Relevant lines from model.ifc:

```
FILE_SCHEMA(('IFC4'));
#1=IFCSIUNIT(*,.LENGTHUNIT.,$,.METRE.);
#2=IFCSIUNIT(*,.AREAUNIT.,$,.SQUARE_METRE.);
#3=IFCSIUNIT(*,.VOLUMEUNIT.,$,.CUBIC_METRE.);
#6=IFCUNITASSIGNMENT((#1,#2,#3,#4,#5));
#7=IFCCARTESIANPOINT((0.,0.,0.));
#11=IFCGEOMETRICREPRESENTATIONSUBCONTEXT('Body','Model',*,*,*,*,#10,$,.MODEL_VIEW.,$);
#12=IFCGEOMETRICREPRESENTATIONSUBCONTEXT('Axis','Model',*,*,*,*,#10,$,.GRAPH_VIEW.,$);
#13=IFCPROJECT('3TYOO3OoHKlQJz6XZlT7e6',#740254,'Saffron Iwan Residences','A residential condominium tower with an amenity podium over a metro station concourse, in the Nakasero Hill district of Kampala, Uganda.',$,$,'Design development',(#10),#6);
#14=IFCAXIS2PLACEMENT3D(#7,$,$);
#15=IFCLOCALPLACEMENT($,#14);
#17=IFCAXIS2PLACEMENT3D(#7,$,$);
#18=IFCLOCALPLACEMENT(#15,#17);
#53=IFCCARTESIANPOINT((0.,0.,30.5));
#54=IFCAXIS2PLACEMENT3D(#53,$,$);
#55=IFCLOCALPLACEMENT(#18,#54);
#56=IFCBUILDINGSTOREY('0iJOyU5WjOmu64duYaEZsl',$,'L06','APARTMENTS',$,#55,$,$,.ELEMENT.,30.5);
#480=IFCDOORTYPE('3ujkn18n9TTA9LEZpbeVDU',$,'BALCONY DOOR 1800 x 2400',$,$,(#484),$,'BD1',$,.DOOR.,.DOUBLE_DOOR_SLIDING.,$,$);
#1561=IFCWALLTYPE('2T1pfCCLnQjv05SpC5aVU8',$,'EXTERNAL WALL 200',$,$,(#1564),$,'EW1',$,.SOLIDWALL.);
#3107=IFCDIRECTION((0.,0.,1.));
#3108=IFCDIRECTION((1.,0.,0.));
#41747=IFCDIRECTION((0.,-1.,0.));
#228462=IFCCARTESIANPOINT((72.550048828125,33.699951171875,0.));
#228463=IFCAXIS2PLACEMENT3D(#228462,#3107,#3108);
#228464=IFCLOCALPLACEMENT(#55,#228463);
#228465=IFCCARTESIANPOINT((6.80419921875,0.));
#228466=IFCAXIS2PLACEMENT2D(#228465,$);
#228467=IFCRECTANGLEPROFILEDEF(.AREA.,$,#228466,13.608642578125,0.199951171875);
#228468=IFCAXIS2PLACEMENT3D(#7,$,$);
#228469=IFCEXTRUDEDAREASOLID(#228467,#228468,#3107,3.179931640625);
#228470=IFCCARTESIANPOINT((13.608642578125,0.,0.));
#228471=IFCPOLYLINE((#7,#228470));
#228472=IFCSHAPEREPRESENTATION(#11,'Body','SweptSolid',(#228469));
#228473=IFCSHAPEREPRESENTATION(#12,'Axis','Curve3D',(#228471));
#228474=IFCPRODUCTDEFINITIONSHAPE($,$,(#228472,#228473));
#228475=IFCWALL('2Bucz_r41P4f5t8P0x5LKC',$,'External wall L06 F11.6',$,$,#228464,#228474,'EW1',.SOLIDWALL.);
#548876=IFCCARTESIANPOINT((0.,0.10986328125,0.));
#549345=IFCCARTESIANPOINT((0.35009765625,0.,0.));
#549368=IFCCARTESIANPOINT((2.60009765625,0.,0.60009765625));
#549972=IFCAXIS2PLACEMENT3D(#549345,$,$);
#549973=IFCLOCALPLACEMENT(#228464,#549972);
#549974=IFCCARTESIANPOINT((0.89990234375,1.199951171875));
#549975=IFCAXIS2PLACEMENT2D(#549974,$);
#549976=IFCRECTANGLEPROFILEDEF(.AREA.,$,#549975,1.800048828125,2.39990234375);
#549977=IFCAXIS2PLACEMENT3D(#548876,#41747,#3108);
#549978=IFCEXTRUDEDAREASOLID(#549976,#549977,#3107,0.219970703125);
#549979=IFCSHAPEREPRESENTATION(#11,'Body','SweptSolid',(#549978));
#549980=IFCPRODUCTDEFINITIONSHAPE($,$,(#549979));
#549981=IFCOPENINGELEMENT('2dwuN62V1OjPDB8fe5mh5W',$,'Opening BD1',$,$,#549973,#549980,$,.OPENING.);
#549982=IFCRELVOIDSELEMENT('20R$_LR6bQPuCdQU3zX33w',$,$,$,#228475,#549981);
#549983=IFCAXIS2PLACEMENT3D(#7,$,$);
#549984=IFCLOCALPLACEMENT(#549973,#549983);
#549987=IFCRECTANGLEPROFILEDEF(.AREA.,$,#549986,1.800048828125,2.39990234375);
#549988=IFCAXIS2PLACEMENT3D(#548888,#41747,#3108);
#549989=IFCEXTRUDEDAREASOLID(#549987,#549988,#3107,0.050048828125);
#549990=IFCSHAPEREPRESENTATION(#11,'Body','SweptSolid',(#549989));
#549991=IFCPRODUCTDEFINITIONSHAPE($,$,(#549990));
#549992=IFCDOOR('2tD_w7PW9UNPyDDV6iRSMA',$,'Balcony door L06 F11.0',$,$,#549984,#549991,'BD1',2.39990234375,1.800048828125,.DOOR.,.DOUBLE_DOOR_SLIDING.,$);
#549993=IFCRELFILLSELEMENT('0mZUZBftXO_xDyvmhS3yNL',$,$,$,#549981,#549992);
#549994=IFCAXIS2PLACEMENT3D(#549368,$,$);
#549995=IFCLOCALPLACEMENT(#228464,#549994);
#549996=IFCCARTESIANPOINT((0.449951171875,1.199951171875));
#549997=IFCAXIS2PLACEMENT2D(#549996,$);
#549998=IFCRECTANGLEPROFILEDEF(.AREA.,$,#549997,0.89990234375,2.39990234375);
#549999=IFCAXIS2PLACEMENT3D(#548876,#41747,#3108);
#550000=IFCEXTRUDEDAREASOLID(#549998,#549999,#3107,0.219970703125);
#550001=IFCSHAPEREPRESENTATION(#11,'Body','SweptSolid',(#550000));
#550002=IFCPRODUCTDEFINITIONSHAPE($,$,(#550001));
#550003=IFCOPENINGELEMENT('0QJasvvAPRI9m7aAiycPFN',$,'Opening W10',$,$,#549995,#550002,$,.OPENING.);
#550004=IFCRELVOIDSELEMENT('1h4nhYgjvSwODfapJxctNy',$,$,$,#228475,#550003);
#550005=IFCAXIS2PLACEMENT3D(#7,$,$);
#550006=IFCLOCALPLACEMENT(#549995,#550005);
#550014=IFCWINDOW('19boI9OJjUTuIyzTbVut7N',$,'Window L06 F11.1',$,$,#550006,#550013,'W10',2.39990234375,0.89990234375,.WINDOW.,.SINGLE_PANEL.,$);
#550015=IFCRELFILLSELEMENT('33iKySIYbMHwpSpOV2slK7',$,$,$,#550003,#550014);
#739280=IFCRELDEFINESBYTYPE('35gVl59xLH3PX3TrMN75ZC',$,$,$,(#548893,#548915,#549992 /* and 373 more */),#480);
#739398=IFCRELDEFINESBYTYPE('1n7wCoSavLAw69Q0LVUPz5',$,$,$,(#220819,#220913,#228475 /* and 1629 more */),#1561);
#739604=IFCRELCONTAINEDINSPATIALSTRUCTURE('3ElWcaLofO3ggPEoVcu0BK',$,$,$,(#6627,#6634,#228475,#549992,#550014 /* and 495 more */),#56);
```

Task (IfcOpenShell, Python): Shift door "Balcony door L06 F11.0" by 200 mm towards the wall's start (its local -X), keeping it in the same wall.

```python
import ifcopenshell
import ifcopenshell.api.geometry
import ifcopenshell.util.placement
import ifcopenshell.util.unit

model = ifcopenshell.open("model.ifc")
unit_scale = ifcopenshell.util.unit.calculate_unit_scale(model)

door = model.by_id(549992)
opening = door.FillsVoids[0].RelatingOpeningElement
wall = opening.VoidsElements[0].RelatingBuildingElement

wall_matrix = ifcopenshell.util.placement.get_local_placement(wall.ObjectPlacement)
shift = wall_matrix[:3, 0] * -0.2 / unit_scale
before = ifcopenshell.util.placement.get_local_placement(door.ObjectPlacement)[:3, 3].copy()

# The door is placed relative to its opening, so it follows when the opening moves.
matrix = ifcopenshell.util.placement.get_local_placement(opening.ObjectPlacement)
matrix[:3, 3] += shift
ifcopenshell.api.geometry.edit_object_placement(
    model, product=opening, matrix=matrix, is_si=False, should_transform_children=True
)

after = ifcopenshell.util.placement.get_local_placement(door.ObjectPlacement)[:3, 3]
print("door moved by", (after - before).round(3) + 0.0)

model.write("model_edited.ifc")
```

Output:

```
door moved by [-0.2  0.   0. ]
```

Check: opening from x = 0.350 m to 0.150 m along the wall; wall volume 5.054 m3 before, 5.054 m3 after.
